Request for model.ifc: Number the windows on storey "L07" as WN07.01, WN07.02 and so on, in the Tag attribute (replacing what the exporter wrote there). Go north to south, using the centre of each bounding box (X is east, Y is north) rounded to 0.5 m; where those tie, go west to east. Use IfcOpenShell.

First a look at what the model holds.

```python
import ifcopenshell
import ifcopenshell.util.element
import ifcopenshell.util.placement

model = ifcopenshell.open("model.ifc")
print(model.schema)
storey = next(s for s in model.by_type("IfcBuildingStorey") if s.Name == "L07")
windows = [e for e in ifcopenshell.util.element.get_decomposition(storey) if e.is_a("IfcWindow")]
for e in sorted(windows, key=lambda e: e.id()):
    origin = ifcopenshell.util.placement.get_local_placement(e.ObjectPlacement)[:3, 3]
    print(e.id(), e.Tag, e.Name, origin.round(2) + 0.0, sep=" | ")
```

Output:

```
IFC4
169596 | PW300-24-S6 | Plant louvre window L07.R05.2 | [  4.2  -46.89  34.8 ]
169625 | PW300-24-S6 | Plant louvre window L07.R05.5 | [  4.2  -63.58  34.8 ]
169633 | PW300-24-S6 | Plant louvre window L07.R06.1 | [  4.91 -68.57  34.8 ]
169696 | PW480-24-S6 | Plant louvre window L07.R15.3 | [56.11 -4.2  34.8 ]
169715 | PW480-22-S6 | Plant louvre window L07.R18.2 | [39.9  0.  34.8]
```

```python
import ifcopenshell
import ifcopenshell.geom
import ifcopenshell.util.element
import ifcopenshell.util.shape

model = ifcopenshell.open("model.ifc")
settings = ifcopenshell.geom.settings()
settings.set("use-world-coords", True)


def centre(element):
    shape = ifcopenshell.geom.create_shape(settings, element)
    return ifcopenshell.util.shape.get_bbox_centroid(shape.geometry)


storey = next(s for s in model.by_type("IfcBuildingStorey") if s.Name == "L07")
windows = [e for e in ifcopenshell.util.element.get_decomposition(storey) if e.is_a("IfcWindow")]

# Insertion points can sit at a corner or the storey origin, so sort by the geometry (in metres).
centres = {e: centre(e) for e in windows}
windows.sort(key=lambda e: (-round(centres[e][1] / 0.5), centres[e][0]))

for i, e in enumerate(windows, start=1):
    number = f"WN07.{i:02d}"
    e.Tag = number
    print(e.id(), number)

model.write("model_updated.ifc")
```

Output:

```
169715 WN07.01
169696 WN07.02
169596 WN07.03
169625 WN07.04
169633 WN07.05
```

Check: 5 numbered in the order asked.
